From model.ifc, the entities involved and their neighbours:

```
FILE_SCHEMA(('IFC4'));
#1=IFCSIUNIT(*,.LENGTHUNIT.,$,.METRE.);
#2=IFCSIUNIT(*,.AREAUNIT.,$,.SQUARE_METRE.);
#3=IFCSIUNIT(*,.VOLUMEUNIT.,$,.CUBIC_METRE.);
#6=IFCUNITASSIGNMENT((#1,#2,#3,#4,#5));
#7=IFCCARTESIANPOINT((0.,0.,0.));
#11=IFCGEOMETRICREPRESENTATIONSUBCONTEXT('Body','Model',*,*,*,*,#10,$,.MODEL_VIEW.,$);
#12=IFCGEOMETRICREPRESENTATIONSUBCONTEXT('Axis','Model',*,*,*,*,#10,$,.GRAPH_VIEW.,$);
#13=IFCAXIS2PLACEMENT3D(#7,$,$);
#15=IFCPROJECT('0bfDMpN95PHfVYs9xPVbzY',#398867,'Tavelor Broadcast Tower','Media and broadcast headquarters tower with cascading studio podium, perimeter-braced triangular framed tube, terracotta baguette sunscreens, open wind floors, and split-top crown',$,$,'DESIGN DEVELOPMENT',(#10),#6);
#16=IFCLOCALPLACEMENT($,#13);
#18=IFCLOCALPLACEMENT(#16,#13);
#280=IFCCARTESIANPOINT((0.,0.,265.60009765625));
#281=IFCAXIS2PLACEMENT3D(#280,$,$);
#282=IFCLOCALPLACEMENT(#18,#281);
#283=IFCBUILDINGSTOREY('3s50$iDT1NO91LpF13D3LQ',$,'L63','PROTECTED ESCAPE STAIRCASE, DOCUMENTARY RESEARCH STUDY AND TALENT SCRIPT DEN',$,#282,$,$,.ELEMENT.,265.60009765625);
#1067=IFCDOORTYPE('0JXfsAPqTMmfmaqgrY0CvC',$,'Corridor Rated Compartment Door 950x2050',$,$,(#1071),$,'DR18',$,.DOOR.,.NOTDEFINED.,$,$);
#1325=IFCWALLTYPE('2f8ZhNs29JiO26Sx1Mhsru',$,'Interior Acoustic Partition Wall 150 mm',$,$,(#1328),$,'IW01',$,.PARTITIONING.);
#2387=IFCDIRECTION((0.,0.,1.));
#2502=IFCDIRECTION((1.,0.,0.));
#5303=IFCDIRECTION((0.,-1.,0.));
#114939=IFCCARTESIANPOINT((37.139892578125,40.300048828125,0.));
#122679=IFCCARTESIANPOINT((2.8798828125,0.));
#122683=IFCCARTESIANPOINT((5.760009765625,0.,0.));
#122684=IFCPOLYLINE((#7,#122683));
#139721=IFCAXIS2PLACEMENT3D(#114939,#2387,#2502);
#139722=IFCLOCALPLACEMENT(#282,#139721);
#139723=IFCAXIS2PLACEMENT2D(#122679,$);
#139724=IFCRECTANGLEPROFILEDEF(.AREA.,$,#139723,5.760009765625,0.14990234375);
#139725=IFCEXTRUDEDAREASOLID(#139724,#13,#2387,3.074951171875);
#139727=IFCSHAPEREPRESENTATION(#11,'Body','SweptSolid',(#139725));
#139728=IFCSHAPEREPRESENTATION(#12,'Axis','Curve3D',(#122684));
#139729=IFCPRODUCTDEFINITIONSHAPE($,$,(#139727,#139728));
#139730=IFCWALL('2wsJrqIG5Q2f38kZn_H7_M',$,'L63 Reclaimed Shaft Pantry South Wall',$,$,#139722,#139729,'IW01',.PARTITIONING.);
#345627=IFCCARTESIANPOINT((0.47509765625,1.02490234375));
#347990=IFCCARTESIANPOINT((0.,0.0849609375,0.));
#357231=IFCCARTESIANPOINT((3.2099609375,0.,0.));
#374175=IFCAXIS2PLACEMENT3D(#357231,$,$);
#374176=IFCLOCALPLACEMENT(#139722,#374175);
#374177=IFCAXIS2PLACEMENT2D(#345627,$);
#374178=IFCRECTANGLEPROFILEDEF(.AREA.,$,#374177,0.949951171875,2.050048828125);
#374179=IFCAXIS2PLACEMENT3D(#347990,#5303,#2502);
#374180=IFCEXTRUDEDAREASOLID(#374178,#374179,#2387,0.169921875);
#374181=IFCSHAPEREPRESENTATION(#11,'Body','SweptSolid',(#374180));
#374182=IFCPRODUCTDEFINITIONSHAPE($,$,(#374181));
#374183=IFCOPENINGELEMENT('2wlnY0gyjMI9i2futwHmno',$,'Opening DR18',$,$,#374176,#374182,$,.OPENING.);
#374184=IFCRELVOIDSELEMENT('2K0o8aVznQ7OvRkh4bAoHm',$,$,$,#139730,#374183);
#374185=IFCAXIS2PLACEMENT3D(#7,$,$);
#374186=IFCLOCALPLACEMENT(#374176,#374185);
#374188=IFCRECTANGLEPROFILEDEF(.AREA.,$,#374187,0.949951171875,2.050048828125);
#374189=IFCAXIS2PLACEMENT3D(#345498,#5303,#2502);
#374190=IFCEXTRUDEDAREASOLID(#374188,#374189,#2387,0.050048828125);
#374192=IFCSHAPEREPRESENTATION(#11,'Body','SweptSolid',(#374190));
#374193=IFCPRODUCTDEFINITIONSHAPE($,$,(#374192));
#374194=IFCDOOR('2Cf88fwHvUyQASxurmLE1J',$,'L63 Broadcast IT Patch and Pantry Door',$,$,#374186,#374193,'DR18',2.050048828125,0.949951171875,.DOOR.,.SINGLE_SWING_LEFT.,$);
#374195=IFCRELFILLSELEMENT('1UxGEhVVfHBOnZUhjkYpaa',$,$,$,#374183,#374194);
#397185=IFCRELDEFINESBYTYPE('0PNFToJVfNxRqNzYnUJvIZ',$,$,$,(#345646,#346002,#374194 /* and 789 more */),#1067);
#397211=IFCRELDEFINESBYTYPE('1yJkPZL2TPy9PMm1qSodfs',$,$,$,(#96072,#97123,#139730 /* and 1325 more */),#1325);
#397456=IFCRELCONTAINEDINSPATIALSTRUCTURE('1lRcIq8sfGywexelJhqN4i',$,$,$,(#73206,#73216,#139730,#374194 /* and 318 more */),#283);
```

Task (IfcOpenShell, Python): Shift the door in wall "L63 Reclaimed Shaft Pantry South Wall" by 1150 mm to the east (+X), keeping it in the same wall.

```python
import ifcopenshell
import ifcopenshell.api.geometry
import ifcopenshell.util.placement
import ifcopenshell.util.unit

model = ifcopenshell.open("model.ifc")
unit_scale = ifcopenshell.util.unit.calculate_unit_scale(model)

door = model.by_id(374194)
opening = door.FillsVoids[0].RelatingOpeningElement
wall = opening.VoidsElements[0].RelatingBuildingElement

wall_matrix = ifcopenshell.util.placement.get_local_placement(wall.ObjectPlacement)
shift = wall_matrix[:3, 0] * 1.15 / unit_scale
before = ifcopenshell.util.placement.get_local_placement(door.ObjectPlacement)[:3, 3].copy()

# The door is placed relative to its opening, so it follows when the opening moves.
matrix = ifcopenshell.util.placement.get_local_placement(opening.ObjectPlacement)
matrix[:3, 3] += shift
ifcopenshell.api.geometry.edit_object_placement(
    model, product=opening, matrix=matrix, is_si=False, should_transform_children=True
)

after = ifcopenshell.util.placement.get_local_placement(door.ObjectPlacement)[:3, 3]
print("door moved by", (after - before).round(3) + 0.0)

model.write("model_edited.ifc")
```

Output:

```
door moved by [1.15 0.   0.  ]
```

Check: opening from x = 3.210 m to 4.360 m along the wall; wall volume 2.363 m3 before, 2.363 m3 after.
